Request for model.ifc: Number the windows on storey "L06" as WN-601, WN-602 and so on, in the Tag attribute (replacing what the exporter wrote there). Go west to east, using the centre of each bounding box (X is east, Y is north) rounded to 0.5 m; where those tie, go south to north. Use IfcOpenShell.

First a look at what the model holds.

```python
import ifcopenshell
import ifcopenshell.util.element
import ifcopenshell.util.placement

model = ifcopenshell.open("model.ifc")
print(model.schema)
storey = next(s for s in model.by_type("IfcBuildingStorey") if s.Name == "L06")
windows = [e for e in ifcopenshell.util.element.get_decomposition(storey) if e.is_a("IfcWindow")]
for e in sorted(windows, key=lambda e: e.id()):
    origin = ifcopenshell.util.placement.get_local_placement(e.ObjectPlacement)[:3, 3]
    print(e.id(), e.Tag, e.Name, origin.round(2) + 0.0, sep=" | ")
```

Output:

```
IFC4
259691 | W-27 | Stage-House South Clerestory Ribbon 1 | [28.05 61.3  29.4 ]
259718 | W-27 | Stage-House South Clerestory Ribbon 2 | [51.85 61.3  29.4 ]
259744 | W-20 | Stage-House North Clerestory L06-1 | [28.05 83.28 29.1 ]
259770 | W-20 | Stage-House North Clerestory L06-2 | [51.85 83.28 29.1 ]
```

```python
import ifcopenshell
import ifcopenshell.geom
import ifcopenshell.util.element
import ifcopenshell.util.shape

model = ifcopenshell.open("model.ifc")
settings = ifcopenshell.geom.settings()
settings.set("use-world-coords", True)


def centre(element):
    shape = ifcopenshell.geom.create_shape(settings, element)
    return ifcopenshell.util.shape.get_bbox_centroid(shape.geometry)


storey = next(s for s in model.by_type("IfcBuildingStorey") if s.Name == "L06")
windows = [e for e in ifcopenshell.util.element.get_decomposition(storey) if e.is_a("IfcWindow")]

# Insertion points can sit at a corner or the storey origin, so sort by the geometry (in metres).
centres = {e: centre(e) for e in windows}
windows.sort(key=lambda e: (round(centres[e][0] / 0.5), centres[e][1]))

for i, e in enumerate(windows, start=1):
    number = f"WN-6{i:02d}"
    e.Tag = number
    print(e.id(), number)

model.write("model_v2.ifc")
```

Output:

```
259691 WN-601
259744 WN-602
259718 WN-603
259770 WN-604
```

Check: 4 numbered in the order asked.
